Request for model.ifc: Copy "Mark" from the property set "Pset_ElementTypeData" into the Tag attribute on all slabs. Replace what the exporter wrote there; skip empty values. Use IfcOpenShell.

First a look at what the model holds.

```python
import ifcopenshell
import ifcopenshell.util.element

model = ifcopenshell.open("model.ifc")
print(model.schema)
slabs = model.by_type("IfcSlab")
print(len(slabs), "slabs")
for e in slabs[:8]:
    source = ifcopenshell.util.element.get_pset(e, "Pset_ElementTypeData", "Mark")
    target = e.Tag
    print(e.id(), repr(source), repr(target), sep=" | ")
```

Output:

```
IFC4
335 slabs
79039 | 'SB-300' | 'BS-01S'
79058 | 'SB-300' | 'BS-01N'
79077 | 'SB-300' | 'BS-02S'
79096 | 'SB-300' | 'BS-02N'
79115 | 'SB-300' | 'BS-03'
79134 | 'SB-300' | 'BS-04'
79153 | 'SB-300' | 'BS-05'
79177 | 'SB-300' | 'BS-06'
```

```python
import ifcopenshell
import ifcopenshell.util.element

model = ifcopenshell.open("model.ifc")

count = 0
for e in model.by_type("IfcSlab"):
    value = ifcopenshell.util.element.get_pset(e, "Pset_ElementTypeData", "Mark")
    current = e.Tag
    if not value or not value.strip() or current == value:
        continue
    e.Tag = value
    count += 1

print(count, "slabs updated")

model.write("model-out.ifc")
```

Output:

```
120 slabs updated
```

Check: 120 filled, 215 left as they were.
